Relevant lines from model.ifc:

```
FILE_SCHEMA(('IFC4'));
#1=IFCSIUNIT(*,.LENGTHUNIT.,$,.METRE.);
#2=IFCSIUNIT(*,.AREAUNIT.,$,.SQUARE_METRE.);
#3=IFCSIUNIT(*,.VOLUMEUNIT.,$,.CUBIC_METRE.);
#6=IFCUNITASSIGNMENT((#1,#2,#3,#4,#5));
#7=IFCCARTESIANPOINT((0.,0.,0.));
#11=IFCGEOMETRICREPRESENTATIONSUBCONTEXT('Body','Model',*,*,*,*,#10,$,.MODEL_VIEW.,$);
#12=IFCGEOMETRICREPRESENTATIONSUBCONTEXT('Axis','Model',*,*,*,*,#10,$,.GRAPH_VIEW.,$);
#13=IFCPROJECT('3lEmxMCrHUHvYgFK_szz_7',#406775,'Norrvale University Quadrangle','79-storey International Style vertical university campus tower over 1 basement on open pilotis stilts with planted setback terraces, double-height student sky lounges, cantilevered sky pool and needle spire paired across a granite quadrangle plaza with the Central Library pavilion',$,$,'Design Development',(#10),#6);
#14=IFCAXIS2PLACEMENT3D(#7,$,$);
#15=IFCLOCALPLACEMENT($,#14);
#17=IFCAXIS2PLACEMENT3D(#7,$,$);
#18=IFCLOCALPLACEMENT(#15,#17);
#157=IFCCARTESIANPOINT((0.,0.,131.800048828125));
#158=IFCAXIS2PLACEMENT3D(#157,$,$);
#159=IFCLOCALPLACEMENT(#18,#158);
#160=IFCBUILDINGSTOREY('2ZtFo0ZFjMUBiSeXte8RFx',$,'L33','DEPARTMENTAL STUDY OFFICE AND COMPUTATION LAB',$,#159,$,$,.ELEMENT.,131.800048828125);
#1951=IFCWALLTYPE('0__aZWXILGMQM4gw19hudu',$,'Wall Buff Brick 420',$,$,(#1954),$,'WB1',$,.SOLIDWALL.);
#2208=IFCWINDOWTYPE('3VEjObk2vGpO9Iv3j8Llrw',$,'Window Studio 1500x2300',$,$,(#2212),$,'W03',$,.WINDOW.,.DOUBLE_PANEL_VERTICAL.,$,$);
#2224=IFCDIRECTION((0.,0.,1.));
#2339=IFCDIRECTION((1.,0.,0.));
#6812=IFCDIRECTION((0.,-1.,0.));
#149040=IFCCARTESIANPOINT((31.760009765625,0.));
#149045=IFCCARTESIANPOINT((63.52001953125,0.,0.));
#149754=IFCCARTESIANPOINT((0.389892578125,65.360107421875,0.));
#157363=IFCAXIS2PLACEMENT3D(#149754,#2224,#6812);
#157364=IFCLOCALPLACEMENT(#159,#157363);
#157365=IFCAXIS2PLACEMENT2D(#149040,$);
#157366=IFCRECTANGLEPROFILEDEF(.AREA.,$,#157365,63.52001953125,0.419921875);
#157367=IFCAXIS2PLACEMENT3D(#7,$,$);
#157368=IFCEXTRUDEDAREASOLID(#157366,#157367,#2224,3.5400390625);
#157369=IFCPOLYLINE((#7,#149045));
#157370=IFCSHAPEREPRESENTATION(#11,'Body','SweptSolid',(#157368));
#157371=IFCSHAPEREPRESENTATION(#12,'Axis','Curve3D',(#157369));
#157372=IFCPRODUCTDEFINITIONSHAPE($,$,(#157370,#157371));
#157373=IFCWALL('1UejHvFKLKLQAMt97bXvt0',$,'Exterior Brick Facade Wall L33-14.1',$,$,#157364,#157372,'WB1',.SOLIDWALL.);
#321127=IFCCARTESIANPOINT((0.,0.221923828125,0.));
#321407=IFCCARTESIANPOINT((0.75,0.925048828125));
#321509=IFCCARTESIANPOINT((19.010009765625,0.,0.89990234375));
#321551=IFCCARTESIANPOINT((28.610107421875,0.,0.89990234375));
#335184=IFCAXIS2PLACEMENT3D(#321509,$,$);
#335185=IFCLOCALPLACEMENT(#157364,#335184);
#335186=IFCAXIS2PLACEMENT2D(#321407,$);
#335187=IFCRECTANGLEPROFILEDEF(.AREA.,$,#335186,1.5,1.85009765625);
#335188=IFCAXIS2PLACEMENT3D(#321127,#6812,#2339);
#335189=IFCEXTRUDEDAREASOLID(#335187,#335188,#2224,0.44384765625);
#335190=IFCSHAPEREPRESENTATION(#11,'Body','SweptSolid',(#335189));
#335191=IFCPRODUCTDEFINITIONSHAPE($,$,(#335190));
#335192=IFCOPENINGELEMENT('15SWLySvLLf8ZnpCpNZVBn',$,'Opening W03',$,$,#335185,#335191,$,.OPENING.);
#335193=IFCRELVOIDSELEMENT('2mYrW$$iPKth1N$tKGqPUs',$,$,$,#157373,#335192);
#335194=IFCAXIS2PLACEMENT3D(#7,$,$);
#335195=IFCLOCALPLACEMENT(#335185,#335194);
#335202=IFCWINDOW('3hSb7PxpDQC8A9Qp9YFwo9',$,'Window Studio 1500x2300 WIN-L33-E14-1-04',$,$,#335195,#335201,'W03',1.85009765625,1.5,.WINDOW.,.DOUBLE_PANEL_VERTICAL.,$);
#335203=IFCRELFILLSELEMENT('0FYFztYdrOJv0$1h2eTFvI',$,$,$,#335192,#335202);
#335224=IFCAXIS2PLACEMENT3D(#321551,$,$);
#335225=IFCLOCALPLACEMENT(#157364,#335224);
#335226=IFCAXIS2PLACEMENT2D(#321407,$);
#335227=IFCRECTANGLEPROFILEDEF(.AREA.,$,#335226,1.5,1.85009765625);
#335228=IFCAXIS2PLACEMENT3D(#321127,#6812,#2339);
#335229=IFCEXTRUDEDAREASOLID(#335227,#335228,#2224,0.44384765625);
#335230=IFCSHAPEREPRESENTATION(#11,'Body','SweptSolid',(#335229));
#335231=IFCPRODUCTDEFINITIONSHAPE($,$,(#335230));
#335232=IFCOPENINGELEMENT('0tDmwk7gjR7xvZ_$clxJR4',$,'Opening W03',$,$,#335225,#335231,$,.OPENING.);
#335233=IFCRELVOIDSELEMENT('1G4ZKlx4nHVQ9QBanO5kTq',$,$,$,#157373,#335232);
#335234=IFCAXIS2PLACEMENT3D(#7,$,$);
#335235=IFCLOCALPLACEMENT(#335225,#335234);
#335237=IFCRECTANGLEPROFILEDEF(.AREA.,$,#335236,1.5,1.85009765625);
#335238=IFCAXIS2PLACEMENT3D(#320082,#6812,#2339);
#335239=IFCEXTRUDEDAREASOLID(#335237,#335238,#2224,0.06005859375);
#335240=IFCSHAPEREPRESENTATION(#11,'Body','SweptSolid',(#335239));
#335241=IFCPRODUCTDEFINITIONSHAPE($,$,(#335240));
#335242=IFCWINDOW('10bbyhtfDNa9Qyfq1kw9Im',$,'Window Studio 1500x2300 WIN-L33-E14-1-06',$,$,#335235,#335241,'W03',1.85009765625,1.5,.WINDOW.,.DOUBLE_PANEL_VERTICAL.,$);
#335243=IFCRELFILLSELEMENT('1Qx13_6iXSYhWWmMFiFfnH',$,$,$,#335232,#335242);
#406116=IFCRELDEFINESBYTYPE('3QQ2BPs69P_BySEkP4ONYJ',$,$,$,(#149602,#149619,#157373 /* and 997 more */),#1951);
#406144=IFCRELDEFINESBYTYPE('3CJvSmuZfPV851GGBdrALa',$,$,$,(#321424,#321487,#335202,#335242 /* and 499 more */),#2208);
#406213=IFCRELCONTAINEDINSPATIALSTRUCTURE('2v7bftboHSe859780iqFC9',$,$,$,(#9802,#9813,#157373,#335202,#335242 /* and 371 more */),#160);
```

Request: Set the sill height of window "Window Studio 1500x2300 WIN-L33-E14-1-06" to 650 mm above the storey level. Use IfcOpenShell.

```python
import numpy as np
import ifcopenshell
import ifcopenshell.api.geometry
import ifcopenshell.geom
import ifcopenshell.util.element
import ifcopenshell.util.placement
import ifcopenshell.util.shape
import ifcopenshell.util.unit

model = ifcopenshell.open("model.ifc")
unit_scale = ifcopenshell.util.unit.calculate_unit_scale(model)

window = model.by_guid("10bbyhtfDNa9Qyfq1kw9Im")
opening = window.FillsVoids[0].RelatingOpeningElement
storey = ifcopenshell.util.element.get_container(window, ifc_class="IfcBuildingStorey")
level = ifcopenshell.util.placement.get_local_placement(storey.ObjectPlacement)[2, 3]

# The opening's origin need not be at the sill, so measure its lowest point.
shape = ifcopenshell.geom.create_shape(ifcopenshell.geom.settings(), opening)
bottom = ifcopenshell.util.shape.get_shape_bottom_elevation(shape, shape.geometry) / unit_scale
dz = level + 0.65 / unit_scale - bottom

shift = np.array([0.0, 0.0, dz])
# The window is placed relative to its opening, so it follows when the opening moves.
matrix = ifcopenshell.util.placement.get_local_placement(opening.ObjectPlacement)
matrix[:3, 3] += shift
ifcopenshell.api.geometry.edit_object_placement(
    model, product=opening, matrix=matrix, is_si=False, should_transform_children=True
)

print(f"moved by {dz * unit_scale:+.3f} m")

model.write("model_updated.ifc")
```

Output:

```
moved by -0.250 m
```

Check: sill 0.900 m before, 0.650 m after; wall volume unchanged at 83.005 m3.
